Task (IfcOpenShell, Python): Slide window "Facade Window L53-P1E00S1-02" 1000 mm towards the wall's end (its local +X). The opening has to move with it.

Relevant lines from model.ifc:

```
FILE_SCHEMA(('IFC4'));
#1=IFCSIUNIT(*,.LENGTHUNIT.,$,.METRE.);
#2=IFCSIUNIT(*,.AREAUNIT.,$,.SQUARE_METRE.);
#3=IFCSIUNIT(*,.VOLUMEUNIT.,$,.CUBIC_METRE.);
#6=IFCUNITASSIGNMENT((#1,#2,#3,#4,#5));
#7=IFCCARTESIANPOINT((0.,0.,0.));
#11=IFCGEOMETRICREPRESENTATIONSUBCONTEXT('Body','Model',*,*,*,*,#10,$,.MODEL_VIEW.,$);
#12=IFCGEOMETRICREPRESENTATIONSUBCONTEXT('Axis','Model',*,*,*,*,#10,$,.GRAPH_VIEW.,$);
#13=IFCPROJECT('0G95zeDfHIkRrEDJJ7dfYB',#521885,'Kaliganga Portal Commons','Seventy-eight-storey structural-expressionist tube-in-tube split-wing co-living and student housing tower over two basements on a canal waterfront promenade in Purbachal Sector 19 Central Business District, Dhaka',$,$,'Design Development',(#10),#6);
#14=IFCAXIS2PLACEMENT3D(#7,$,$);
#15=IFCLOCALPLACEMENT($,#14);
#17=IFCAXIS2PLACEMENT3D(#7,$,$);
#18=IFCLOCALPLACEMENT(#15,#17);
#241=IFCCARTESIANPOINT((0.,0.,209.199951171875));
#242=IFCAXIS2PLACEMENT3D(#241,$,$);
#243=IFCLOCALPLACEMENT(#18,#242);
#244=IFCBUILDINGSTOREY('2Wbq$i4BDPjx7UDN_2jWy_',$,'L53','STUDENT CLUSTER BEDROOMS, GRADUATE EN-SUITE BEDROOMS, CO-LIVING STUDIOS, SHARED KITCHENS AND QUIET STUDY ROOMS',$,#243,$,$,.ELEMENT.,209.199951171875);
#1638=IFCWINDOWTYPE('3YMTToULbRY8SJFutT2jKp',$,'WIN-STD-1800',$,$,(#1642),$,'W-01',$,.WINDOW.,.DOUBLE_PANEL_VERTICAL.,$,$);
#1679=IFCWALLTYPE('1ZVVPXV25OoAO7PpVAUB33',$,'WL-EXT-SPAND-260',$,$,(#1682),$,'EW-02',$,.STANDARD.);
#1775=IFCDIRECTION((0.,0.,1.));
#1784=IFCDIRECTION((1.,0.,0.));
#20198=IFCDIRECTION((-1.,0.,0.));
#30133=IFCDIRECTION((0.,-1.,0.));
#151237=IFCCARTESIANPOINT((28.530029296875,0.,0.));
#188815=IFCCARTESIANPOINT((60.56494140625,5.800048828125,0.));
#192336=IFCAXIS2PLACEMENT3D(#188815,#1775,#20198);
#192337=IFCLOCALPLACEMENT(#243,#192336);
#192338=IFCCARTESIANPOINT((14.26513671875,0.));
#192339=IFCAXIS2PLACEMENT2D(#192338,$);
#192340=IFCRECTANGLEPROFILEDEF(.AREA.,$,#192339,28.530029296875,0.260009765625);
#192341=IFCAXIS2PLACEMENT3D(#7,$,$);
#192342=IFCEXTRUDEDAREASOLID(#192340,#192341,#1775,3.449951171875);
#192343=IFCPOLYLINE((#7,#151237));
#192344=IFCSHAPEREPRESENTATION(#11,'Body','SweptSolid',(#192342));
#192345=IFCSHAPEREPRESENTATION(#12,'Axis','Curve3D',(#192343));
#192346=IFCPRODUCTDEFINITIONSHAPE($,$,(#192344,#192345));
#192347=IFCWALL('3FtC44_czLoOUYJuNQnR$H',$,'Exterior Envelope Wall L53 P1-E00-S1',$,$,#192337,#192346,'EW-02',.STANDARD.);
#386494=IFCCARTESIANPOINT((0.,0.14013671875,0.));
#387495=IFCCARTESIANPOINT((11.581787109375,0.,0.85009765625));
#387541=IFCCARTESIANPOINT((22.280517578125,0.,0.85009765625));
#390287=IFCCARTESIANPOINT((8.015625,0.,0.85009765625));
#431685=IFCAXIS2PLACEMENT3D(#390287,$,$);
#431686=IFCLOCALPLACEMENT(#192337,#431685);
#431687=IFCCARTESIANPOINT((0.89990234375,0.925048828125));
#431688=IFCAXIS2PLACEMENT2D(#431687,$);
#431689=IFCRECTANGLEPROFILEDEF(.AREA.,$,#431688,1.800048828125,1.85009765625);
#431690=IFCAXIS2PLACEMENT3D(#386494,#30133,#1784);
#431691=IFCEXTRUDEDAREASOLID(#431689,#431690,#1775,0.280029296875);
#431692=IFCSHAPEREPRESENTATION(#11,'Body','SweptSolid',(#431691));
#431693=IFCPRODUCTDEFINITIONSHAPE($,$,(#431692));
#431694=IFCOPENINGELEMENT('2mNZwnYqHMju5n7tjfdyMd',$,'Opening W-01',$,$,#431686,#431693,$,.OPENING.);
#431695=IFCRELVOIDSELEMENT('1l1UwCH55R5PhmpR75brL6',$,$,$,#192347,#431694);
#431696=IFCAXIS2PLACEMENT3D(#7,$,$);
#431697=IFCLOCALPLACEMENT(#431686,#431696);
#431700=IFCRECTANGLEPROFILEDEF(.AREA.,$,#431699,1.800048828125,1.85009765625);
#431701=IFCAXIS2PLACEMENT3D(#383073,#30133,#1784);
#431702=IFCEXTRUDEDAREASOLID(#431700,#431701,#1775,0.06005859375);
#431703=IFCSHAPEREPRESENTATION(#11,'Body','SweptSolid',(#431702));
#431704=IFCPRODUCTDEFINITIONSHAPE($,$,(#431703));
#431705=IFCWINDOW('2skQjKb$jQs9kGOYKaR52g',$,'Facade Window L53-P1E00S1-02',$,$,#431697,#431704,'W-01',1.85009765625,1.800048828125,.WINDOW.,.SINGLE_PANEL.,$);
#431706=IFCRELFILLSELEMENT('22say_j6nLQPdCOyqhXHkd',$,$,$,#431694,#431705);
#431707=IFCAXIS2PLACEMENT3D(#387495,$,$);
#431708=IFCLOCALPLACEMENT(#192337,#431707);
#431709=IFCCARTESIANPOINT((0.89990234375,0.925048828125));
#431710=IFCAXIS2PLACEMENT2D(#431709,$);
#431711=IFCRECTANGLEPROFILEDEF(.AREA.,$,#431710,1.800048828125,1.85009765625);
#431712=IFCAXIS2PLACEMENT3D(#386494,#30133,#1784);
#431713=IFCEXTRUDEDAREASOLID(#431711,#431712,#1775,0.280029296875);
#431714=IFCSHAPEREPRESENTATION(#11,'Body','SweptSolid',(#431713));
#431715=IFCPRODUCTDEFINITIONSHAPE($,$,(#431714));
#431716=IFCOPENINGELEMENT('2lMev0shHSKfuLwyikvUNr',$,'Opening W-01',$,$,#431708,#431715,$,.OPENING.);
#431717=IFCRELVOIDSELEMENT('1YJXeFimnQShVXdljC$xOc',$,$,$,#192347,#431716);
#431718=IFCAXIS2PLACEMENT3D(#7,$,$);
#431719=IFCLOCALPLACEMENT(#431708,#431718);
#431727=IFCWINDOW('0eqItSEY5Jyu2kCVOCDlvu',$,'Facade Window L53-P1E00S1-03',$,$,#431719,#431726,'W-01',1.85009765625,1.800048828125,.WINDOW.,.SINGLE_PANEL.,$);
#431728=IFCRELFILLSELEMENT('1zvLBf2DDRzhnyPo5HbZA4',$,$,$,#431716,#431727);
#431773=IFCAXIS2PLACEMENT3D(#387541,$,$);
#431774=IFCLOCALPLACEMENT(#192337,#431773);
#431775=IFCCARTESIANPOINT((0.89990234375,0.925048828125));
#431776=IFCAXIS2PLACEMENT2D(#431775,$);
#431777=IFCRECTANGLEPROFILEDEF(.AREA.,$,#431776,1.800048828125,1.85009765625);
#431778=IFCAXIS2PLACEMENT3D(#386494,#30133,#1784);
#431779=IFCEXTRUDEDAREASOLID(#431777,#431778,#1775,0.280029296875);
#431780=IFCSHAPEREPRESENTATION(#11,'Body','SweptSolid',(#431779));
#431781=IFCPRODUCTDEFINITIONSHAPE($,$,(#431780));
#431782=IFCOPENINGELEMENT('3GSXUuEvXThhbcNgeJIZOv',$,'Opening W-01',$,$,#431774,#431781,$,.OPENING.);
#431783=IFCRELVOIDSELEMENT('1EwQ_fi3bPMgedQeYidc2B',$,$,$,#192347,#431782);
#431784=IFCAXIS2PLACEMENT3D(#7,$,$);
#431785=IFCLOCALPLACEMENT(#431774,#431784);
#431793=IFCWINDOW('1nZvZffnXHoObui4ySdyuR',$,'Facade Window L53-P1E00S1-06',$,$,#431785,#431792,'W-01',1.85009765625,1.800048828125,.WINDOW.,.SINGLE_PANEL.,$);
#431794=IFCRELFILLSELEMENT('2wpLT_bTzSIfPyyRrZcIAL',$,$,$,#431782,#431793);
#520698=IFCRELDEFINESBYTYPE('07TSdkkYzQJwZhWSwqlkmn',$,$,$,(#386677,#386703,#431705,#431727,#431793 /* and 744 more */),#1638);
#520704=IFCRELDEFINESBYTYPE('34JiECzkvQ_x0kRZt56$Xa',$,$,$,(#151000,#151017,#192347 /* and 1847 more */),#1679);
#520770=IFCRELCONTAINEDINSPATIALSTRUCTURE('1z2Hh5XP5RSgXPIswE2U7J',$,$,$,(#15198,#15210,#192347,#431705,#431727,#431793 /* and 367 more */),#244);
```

```python
import ifcopenshell
import ifcopenshell.api.geometry
import ifcopenshell.util.placement

model = ifcopenshell.open("model.ifc")

window = model.by_id(431705)
opening = window.FillsVoids[0].RelatingOpeningElement
wall = opening.VoidsElements[0].RelatingBuildingElement

wall_matrix = ifcopenshell.util.placement.get_local_placement(wall.ObjectPlacement)
shift = wall_matrix[:3, 0] * 1.0
before = ifcopenshell.util.placement.get_local_placement(window.ObjectPlacement)[:3, 3].copy()

# The window is placed relative to its opening, so it follows when the opening moves.
matrix = ifcopenshell.util.placement.get_local_placement(opening.ObjectPlacement)
matrix[:3, 3] += shift
ifcopenshell.api.geometry.edit_object_placement(
    model, product=opening, matrix=matrix, is_si=False, should_transform_children=True
)

after = ifcopenshell.util.placement.get_local_placement(window.ObjectPlacement)[:3, 3]
print("window moved by", (after - before).round(3) + 0.0)

model.write("model_edited.ifc")
```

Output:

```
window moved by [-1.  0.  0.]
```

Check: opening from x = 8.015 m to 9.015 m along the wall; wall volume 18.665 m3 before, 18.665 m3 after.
